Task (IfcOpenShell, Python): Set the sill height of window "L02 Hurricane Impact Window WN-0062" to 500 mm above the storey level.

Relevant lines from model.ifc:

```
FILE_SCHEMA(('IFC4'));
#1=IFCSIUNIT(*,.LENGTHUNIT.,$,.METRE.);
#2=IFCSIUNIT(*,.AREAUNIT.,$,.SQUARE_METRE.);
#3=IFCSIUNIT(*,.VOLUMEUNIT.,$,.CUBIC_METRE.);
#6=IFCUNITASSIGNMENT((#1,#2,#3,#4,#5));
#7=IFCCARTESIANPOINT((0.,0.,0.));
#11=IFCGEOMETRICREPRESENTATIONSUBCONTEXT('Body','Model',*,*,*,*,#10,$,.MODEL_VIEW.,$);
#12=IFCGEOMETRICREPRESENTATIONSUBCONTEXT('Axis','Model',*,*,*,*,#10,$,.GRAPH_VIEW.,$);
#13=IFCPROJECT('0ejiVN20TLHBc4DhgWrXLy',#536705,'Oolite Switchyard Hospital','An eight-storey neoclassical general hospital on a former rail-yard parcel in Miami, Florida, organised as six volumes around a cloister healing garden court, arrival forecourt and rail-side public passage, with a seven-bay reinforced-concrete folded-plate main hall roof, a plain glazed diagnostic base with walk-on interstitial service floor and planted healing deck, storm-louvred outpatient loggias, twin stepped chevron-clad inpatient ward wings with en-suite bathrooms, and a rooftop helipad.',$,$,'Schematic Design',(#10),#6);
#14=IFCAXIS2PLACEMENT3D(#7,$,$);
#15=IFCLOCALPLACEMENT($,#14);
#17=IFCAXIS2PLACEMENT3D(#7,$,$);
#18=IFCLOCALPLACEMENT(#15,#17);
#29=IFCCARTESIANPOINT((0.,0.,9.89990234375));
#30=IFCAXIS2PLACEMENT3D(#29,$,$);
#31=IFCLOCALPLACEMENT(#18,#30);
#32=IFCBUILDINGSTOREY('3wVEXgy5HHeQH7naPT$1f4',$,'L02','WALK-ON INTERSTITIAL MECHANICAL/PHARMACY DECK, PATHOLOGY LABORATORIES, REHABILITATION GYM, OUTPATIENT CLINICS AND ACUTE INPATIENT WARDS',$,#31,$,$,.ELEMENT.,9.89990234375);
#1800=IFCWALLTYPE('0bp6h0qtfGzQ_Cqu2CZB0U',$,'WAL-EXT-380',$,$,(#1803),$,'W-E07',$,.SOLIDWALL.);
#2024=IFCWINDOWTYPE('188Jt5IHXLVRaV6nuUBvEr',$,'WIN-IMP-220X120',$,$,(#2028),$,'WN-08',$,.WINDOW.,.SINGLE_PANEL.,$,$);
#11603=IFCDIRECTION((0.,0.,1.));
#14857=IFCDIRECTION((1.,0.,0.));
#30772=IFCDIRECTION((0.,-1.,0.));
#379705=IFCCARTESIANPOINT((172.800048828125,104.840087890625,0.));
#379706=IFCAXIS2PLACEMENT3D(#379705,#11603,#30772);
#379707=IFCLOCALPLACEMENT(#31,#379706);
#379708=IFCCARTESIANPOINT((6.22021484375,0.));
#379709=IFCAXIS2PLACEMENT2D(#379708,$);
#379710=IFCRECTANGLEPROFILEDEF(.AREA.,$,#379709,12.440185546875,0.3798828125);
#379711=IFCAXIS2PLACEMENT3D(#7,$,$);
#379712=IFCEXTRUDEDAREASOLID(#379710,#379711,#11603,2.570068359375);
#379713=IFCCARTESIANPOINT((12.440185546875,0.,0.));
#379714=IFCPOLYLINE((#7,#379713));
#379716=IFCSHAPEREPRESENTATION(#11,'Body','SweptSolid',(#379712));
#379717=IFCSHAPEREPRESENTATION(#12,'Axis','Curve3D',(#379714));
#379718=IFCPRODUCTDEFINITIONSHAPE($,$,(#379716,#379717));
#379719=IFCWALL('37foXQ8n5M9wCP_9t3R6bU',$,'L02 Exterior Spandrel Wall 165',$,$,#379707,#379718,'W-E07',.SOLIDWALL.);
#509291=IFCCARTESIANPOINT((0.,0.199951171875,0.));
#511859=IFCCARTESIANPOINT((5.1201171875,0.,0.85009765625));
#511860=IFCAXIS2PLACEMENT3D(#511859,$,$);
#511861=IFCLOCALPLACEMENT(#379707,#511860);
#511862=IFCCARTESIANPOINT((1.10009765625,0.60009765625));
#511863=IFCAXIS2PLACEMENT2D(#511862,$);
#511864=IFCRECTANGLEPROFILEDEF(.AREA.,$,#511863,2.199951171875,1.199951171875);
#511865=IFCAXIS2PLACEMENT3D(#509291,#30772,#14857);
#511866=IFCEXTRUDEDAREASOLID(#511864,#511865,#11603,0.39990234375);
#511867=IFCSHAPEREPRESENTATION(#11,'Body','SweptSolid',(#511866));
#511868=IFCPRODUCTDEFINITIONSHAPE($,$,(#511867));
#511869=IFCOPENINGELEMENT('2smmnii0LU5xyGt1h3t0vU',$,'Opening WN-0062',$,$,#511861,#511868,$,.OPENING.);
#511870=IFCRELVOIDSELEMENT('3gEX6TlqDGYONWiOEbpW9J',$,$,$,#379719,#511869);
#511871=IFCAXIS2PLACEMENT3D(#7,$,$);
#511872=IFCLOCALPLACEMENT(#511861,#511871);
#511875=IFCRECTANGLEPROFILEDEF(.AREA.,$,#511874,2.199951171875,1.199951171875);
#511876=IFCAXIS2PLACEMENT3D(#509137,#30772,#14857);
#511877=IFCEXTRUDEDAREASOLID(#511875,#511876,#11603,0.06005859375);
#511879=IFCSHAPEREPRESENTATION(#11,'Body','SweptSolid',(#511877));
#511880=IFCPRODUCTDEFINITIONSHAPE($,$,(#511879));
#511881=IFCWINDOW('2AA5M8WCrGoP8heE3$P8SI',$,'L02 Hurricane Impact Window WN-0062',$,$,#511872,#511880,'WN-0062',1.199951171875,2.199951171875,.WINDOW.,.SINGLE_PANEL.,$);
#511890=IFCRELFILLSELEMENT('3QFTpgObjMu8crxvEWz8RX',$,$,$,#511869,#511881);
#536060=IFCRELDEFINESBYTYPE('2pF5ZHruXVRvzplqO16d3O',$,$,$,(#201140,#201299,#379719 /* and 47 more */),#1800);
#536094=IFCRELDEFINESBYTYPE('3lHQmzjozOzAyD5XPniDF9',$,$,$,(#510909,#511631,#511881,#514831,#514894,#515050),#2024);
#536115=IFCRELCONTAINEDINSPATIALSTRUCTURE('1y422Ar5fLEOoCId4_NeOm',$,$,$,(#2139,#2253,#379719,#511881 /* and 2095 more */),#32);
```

```python
import numpy as np
import ifcopenshell
import ifcopenshell.api.geometry
import ifcopenshell.geom
import ifcopenshell.util.element
import ifcopenshell.util.placement
import ifcopenshell.util.shape
import ifcopenshell.util.unit

model = ifcopenshell.open("model.ifc")
unit_scale = ifcopenshell.util.unit.calculate_unit_scale(model)

window = model.by_guid("2AA5M8WCrGoP8heE3$P8SI")
opening = window.FillsVoids[0].RelatingOpeningElement
storey = ifcopenshell.util.element.get_container(window, ifc_class="IfcBuildingStorey")
level = ifcopenshell.util.placement.get_local_placement(storey.ObjectPlacement)[2, 3]

# The opening's origin need not be at the sill, so measure its lowest point.
shape = ifcopenshell.geom.create_shape(ifcopenshell.geom.settings(), opening)
bottom = ifcopenshell.util.shape.get_shape_bottom_elevation(shape, shape.geometry) / unit_scale
dz = level + 0.5 - bottom

shift = np.array([0.0, 0.0, dz])
# The window is placed relative to its opening, so it follows when the opening moves.
matrix = ifcopenshell.util.placement.get_local_placement(opening.ObjectPlacement)
matrix[:3, 3] += shift
ifcopenshell.api.geometry.edit_object_placement(
    model, product=opening, matrix=matrix, is_si=False, should_transform_children=True
)

print(f"moved by {dz * unit_scale:+.3f} m")

model.write("model_v2.ifc")
```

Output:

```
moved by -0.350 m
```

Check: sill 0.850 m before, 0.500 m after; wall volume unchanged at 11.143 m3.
